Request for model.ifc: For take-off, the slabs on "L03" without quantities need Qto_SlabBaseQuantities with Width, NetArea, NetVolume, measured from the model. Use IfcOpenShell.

First a look at what the model holds.

```python
import ifcopenshell
import ifcopenshell.util.element
import ifcopenshell.util.unit

model = ifcopenshell.open("model.ifc")
print(model.schema)
for unit_type in ("LENGTHUNIT", "AREAUNIT", "VOLUMEUNIT"):
    print(unit_type, ifcopenshell.util.unit.calculate_unit_scale(model, unit_type))
storey = next(s for s in model.by_type("IfcBuildingStorey") if s.Name == "L03")
slabs = [e for e in ifcopenshell.util.element.get_decomposition(storey) if e.is_a("IfcSlab")]
for e in sorted(slabs, key=lambda e: e.id()):
    print(e.id(), e.is_a(), e.Name, list(ifcopenshell.util.element.get_psets(e, qtos_only=True)), sep=" | ")
```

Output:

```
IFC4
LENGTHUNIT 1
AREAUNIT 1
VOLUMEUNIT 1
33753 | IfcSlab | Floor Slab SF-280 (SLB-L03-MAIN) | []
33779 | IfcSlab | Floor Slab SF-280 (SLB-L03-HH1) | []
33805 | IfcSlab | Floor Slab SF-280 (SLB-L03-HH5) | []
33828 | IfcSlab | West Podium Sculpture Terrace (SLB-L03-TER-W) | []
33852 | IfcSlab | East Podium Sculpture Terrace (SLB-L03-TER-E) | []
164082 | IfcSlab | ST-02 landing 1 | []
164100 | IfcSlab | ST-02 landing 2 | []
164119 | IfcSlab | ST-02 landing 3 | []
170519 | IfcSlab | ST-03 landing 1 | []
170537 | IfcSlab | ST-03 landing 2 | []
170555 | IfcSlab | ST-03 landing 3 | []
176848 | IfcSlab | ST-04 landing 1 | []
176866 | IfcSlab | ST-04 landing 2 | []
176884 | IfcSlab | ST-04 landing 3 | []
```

```python
import ifcopenshell
import ifcopenshell.api.pset
import ifcopenshell.geom
import ifcopenshell.util.element
import ifcopenshell.util.shape
import ifcopenshell.util.unit

model = ifcopenshell.open("model.ifc")
unit_scale = ifcopenshell.util.unit.calculate_unit_scale(model)
area_scale = ifcopenshell.util.unit.calculate_unit_scale(model, "AREAUNIT")
volume_scale = ifcopenshell.util.unit.calculate_unit_scale(model, "VOLUMEUNIT")
settings = ifcopenshell.geom.settings()

storey = next(s for s in model.by_type("IfcBuildingStorey") if s.Name == "L03")
slabs = [e for e in ifcopenshell.util.element.get_decomposition(storey) if e.is_a("IfcSlab")]

for e in sorted(slabs, key=lambda e: e.id()):
    if ifcopenshell.util.element.get_psets(e, qtos_only=True, should_inherit=False):
        continue
    # Geometry comes back in metres, in the element's own axes.
    shape = ifcopenshell.geom.create_shape(settings, e)
    values = {
        "Width": ifcopenshell.util.shape.get_z(shape.geometry) / unit_scale,
        "NetArea": ifcopenshell.util.shape.get_footprint_area(shape.geometry) / area_scale,
        "NetVolume": ifcopenshell.util.shape.get_volume(shape.geometry) / volume_scale,
    }
    qto = ifcopenshell.api.pset.add_qto(model, product=e, name="Qto_SlabBaseQuantities")
    ifcopenshell.api.pset.edit_qto(model, qto=qto, properties=values)
    print(e.id(), {k: round(v, 3) for k, v in values.items()})

model.write("model_edited.ifc")
```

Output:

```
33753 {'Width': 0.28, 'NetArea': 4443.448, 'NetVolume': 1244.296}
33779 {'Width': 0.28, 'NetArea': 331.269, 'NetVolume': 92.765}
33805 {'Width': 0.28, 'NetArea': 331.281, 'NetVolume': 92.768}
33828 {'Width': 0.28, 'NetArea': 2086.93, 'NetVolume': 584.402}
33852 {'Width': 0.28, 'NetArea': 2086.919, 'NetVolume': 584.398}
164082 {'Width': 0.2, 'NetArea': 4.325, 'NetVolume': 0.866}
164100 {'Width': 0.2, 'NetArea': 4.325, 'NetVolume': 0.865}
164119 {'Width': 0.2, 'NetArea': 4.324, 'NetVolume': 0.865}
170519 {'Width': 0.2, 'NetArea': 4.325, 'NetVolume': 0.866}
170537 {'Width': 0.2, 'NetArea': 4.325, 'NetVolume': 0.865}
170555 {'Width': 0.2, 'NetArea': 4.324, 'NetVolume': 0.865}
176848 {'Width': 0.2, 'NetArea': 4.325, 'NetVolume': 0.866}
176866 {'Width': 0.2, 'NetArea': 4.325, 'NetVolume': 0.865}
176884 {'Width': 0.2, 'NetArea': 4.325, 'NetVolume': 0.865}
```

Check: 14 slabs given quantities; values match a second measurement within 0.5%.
